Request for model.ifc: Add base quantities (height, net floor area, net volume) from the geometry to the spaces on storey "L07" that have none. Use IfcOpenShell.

First a look at what the model holds.

```python
import ifcopenshell
import ifcopenshell.util.element
import ifcopenshell.util.unit

model = ifcopenshell.open("model.ifc")
print(model.schema)
for unit_type in ("LENGTHUNIT", "AREAUNIT", "VOLUMEUNIT"):
    print(unit_type, ifcopenshell.util.unit.calculate_unit_scale(model, unit_type))
storey = next(s for s in model.by_type("IfcBuildingStorey") if s.Name == "L07")
spaces = [e for e in ifcopenshell.util.element.get_decomposition(storey) if e.is_a("IfcSpace")]
for e in sorted(spaces, key=lambda e: e.id()):
    print(e.id(), e.is_a(), e.Name, list(ifcopenshell.util.element.get_psets(e, qtos_only=True)), sep=" | ")
```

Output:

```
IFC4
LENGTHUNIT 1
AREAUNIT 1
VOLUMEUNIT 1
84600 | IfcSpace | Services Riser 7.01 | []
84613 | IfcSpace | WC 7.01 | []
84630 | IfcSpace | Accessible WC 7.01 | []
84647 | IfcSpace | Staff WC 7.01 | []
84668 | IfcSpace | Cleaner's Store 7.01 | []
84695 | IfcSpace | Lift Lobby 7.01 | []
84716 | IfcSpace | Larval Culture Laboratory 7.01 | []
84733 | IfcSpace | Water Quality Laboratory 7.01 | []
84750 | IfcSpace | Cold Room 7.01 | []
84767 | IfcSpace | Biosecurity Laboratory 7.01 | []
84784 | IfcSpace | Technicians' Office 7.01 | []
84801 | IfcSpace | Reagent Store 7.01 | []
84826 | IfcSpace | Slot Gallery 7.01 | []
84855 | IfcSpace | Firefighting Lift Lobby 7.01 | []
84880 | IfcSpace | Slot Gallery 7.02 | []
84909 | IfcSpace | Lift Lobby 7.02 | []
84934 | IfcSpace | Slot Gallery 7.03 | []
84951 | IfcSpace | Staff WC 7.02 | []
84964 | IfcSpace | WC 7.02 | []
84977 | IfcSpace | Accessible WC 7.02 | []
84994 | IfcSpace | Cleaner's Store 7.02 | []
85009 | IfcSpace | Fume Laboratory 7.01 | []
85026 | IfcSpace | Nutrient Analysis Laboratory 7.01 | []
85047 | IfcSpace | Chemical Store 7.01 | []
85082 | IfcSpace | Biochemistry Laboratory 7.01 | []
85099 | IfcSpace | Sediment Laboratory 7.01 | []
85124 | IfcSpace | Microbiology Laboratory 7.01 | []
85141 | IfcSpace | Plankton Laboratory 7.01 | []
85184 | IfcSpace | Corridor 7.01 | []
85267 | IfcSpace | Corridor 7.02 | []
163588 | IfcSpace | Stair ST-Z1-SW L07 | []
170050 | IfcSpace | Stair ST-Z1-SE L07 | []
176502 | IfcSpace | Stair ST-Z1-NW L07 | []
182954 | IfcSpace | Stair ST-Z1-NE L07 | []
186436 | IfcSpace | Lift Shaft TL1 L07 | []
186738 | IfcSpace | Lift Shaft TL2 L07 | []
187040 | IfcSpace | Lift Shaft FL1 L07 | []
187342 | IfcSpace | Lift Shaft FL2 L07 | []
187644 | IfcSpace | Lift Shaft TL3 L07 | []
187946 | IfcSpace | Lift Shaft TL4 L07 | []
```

```python
import ifcopenshell
import ifcopenshell.api.pset
import ifcopenshell.geom
import ifcopenshell.util.element
import ifcopenshell.util.shape
import ifcopenshell.util.unit

model = ifcopenshell.open("model.ifc")
unit_scale = ifcopenshell.util.unit.calculate_unit_scale(model)
area_scale = ifcopenshell.util.unit.calculate_unit_scale(model, "AREAUNIT")
volume_scale = ifcopenshell.util.unit.calculate_unit_scale(model, "VOLUMEUNIT")
settings = ifcopenshell.geom.settings()

storey = next(s for s in model.by_type("IfcBuildingStorey") if s.Name == "L07")
spaces = [e for e in ifcopenshell.util.element.get_decomposition(storey) if e.is_a("IfcSpace")]

for e in sorted(spaces, key=lambda e: e.id()):
    if ifcopenshell.util.element.get_psets(e, qtos_only=True, should_inherit=False):
        continue
    # Geometry comes back in metres, in the element's own axes.
    shape = ifcopenshell.geom.create_shape(settings, e)
    values = {
        "Height": ifcopenshell.util.shape.get_z(shape.geometry) / unit_scale,
        "NetFloorArea": ifcopenshell.util.shape.get_footprint_area(shape.geometry) / area_scale,
        "NetVolume": ifcopenshell.util.shape.get_volume(shape.geometry) / volume_scale,
    }
    qto = ifcopenshell.api.pset.add_qto(model, product=e, name="Qto_SpaceBaseQuantities")
    ifcopenshell.api.pset.edit_qto(model, qto=qto, properties=values)
    print(e.id(), {k: round(v, 3) for k, v in values.items()})

model.write("model_v2.ifc")
```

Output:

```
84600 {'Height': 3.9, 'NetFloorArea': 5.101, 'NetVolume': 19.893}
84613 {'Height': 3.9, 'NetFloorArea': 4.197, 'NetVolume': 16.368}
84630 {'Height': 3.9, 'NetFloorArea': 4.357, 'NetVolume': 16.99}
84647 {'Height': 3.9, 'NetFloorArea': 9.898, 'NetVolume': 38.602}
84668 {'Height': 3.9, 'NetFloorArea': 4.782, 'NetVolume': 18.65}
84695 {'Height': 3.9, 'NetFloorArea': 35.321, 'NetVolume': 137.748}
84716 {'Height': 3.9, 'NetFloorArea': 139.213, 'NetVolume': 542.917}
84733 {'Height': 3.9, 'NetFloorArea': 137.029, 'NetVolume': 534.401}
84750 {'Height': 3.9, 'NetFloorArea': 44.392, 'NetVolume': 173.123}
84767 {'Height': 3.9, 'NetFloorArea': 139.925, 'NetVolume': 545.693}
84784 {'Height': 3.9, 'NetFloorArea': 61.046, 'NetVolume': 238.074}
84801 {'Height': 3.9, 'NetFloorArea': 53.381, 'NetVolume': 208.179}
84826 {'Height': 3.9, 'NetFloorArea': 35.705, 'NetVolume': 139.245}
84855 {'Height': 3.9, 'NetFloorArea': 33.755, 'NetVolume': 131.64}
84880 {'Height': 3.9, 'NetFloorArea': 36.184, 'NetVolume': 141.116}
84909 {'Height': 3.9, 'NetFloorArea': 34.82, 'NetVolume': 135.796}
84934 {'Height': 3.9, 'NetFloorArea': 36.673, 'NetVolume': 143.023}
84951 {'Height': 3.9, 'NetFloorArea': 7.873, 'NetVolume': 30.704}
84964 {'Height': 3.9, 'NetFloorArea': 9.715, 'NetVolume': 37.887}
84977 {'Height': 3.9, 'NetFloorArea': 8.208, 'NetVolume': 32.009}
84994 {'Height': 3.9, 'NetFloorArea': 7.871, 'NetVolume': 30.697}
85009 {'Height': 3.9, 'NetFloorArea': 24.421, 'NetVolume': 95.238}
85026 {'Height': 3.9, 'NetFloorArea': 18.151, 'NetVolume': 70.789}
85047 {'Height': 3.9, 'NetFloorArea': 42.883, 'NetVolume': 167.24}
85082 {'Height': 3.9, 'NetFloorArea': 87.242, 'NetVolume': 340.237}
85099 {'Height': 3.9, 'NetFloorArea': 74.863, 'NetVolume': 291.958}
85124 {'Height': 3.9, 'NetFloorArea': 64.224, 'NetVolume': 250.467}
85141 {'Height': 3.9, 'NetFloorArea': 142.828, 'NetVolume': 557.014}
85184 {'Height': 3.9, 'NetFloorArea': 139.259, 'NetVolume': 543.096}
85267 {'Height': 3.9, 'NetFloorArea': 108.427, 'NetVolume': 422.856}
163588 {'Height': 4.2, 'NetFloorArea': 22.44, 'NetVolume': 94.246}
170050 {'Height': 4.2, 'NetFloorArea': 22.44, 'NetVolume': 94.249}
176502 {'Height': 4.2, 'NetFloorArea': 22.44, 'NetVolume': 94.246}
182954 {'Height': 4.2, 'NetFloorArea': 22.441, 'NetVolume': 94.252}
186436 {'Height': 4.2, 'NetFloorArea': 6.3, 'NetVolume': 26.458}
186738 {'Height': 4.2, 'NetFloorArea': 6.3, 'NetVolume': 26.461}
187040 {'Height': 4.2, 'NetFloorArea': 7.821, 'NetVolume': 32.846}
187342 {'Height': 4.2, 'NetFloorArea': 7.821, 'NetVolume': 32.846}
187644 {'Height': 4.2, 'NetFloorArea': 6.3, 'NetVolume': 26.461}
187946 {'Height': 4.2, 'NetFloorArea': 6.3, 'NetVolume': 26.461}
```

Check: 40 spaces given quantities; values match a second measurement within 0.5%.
